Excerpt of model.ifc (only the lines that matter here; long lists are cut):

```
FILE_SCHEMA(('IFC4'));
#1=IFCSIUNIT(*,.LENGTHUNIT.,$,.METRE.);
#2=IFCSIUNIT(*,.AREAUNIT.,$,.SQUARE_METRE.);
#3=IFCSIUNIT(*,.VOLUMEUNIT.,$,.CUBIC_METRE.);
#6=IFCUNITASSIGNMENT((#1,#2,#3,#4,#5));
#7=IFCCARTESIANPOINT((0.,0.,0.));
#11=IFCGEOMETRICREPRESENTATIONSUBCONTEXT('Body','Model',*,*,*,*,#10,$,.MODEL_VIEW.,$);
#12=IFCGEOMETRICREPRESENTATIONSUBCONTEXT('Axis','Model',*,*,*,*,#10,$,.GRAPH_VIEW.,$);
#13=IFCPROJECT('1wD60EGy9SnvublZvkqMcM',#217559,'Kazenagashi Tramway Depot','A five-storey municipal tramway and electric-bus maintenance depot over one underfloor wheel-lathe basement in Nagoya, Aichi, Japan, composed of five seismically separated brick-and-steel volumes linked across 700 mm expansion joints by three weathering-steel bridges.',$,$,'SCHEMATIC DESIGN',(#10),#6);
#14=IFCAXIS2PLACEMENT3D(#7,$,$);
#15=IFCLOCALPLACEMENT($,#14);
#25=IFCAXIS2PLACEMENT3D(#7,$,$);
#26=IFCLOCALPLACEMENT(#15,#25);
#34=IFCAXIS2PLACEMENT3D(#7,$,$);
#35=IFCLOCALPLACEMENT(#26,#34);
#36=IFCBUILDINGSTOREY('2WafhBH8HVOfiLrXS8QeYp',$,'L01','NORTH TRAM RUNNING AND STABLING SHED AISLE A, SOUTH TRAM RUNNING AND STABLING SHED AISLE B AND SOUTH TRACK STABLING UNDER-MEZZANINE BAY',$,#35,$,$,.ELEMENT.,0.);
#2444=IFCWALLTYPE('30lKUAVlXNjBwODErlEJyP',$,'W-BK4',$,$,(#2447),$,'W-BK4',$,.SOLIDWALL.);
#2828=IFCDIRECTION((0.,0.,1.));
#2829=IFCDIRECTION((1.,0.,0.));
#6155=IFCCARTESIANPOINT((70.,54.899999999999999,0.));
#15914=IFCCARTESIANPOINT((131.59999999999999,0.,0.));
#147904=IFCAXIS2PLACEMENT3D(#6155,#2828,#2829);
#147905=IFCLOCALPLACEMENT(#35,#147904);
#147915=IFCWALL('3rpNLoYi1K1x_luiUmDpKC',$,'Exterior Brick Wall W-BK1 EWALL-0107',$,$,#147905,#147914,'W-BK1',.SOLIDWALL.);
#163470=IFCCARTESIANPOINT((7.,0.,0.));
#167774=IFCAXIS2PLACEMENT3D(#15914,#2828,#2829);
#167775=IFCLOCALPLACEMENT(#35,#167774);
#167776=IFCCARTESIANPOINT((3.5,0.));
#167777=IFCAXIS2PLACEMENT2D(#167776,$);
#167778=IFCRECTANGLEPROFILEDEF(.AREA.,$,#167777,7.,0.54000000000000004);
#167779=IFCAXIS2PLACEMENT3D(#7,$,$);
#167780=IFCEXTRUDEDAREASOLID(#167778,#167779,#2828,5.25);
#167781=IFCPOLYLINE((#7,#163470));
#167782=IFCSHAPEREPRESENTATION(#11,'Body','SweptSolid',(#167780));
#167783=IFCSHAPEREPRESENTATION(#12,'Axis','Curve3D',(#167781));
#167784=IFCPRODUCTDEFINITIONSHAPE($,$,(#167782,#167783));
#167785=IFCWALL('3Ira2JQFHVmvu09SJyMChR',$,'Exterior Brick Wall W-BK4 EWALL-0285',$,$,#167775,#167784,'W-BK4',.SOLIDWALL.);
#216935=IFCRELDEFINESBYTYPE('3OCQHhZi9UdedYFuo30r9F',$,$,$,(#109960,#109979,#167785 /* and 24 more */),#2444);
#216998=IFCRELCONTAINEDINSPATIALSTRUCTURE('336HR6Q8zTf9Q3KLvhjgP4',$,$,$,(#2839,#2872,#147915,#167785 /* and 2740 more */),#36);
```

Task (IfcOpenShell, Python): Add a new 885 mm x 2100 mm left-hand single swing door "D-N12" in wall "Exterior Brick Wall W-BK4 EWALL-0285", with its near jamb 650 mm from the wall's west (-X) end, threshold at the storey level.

```python
import numpy as np
import ifcopenshell
import ifcopenshell.api.feature
import ifcopenshell.api.geometry
import ifcopenshell.api.root
import ifcopenshell.api.spatial
import ifcopenshell.geom
import ifcopenshell.util.element
import ifcopenshell.util.placement
import ifcopenshell.util.representation
import ifcopenshell.util.shape
import ifcopenshell.util.unit

model = ifcopenshell.open("model.ifc")
unit_scale = ifcopenshell.util.unit.calculate_unit_scale(model)
settings = ifcopenshell.geom.settings()


def volume(element):
    """Net volume in cubic metres, openings subtracted."""
    shape = ifcopenshell.geom.create_shape(settings, element)
    return ifcopenshell.util.shape.get_volume(shape.geometry)


wall = model.by_id(167785)
storey = ifcopenshell.util.element.get_container(wall, ifc_class="IfcBuildingStorey")
context = ifcopenshell.util.representation.get_context(model, "Model", "Body", "MODEL_VIEW")
before = volume(wall)

width, height, from_end, sill = 0.885, 2.1, 0.65, 0.0  # metres

# The wall runs along its own X axis, and the end named is its -X end.
wall_shape = ifcopenshell.geom.create_shape(settings, wall)
x, y, z = ifcopenshell.util.shape.get_vertices(wall_shape.geometry).T
start = x.min() + from_end
face, thickness = float(y.min()), float(y.max() - y.min())
wall_matrix = ifcopenshell.util.placement.get_local_placement(wall.ObjectPlacement)
level = ifcopenshell.util.placement.get_local_placement(storey.ObjectPlacement)[2, 3]


def in_wall(x, y):
    """Placement at x, y metres in the wall's axes, at sill height."""
    matrix = wall_matrix.copy()
    matrix[:, 3] = wall_matrix @ np.array([x / unit_scale, y / unit_scale, 0.0, 1.0])
    matrix[2, 3] = level + sill / unit_scale
    return matrix


# Opening: a box that overshoots both wall faces by 50 mm.
opening = ifcopenshell.api.root.create_entity(model, ifc_class="IfcOpeningElement", predefined_type="OPENING")
box = ifcopenshell.api.geometry.add_wall_representation(
    model, context=context, length=width, height=height, thickness=thickness + 0.1
)
ifcopenshell.api.geometry.assign_representation(model, product=opening, representation=box)
ifcopenshell.api.geometry.edit_object_placement(model, product=opening, matrix=in_wall(start, face - 0.05), is_si=False)
ifcopenshell.api.feature.add_feature(model, feature=opening, element=wall)

door = ifcopenshell.api.root.create_entity(model, ifc_class="IfcDoor", name="D-N12", predefined_type="DOOR")
door.OverallWidth, door.OverallHeight = width / unit_scale, height / unit_scale
door.OperationType = "SINGLE_SWING_LEFT"
body = ifcopenshell.api.geometry.add_door_representation(
    model,
    context=context,
    overall_width=door.OverallWidth,
    overall_height=door.OverallHeight,
    operation_type="SINGLE_SWING_LEFT",
    lining_properties={"LiningDepth": thickness / unit_scale, "ThresholdDepth": thickness / unit_scale},
)
ifcopenshell.api.geometry.assign_representation(model, product=door, representation=body)
ifcopenshell.api.spatial.assign_container(model, products=[door], relating_structure=storey)
ifcopenshell.api.feature.add_filling(model, opening=opening, element=door)

# The lining spans the wall, so the door starts at the wall face.
ifcopenshell.api.geometry.edit_object_placement(model, product=door, matrix=in_wall(start, face), is_si=False)

after = volume(wall)

print(f"wall volume {before:.3f} -> {after:.3f} m3")

model.write("model_v2.ifc")
```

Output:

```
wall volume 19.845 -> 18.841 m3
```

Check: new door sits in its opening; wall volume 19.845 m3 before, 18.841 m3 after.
